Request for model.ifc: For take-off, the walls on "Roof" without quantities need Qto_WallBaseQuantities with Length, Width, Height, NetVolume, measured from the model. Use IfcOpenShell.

First a look at what the model holds.

```python
import ifcopenshell
import ifcopenshell.util.element
import ifcopenshell.util.unit

model = ifcopenshell.open("model.ifc")
print(model.schema)
for unit_type in ("LENGTHUNIT", "AREAUNIT", "VOLUMEUNIT"):
    print(unit_type, ifcopenshell.util.unit.calculate_unit_scale(model, unit_type))
storey = next(s for s in model.by_type("IfcBuildingStorey") if s.Name == "Roof")
walls = [e for e in ifcopenshell.util.element.get_decomposition(storey) if e.is_a("IfcWall")]
for e in sorted(walls, key=lambda e: e.id()):
    print(e.id(), e.is_a(), e.Name, list(ifcopenshell.util.element.get_psets(e, qtos_only=True)), sep=" | ")
```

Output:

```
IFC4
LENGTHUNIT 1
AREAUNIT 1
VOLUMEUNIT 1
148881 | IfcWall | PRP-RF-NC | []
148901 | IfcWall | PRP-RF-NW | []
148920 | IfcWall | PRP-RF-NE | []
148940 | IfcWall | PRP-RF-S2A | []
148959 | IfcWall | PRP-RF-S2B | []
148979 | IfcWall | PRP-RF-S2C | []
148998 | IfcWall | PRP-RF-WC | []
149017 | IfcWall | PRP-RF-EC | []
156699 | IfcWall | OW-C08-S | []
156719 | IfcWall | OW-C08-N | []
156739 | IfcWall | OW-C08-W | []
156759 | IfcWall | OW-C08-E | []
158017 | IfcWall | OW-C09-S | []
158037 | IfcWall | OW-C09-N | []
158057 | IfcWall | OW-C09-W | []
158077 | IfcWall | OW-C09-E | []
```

```python
import ifcopenshell
import ifcopenshell.api.pset
import ifcopenshell.geom
import ifcopenshell.util.element
import ifcopenshell.util.shape
import ifcopenshell.util.unit

model = ifcopenshell.open("model.ifc")
unit_scale = ifcopenshell.util.unit.calculate_unit_scale(model)
volume_scale = ifcopenshell.util.unit.calculate_unit_scale(model, "VOLUMEUNIT")
settings = ifcopenshell.geom.settings()

storey = next(s for s in model.by_type("IfcBuildingStorey") if s.Name == "Roof")
walls = [e for e in ifcopenshell.util.element.get_decomposition(storey) if e.is_a("IfcWall")]

for e in sorted(walls, key=lambda e: e.id()):
    if ifcopenshell.util.element.get_psets(e, qtos_only=True, should_inherit=False):
        continue
    # Geometry comes back in metres, in the element's own axes.
    shape = ifcopenshell.geom.create_shape(settings, e)
    values = {
        "Length": ifcopenshell.util.shape.get_x(shape.geometry) / unit_scale,
        "Width": ifcopenshell.util.shape.get_y(shape.geometry) / unit_scale,
        "Height": ifcopenshell.util.shape.get_z(shape.geometry) / unit_scale,
        "NetVolume": ifcopenshell.util.shape.get_volume(shape.geometry) / volume_scale,
    }
    qto = ifcopenshell.api.pset.add_qto(model, product=e, name="Qto_WallBaseQuantities")
    ifcopenshell.api.pset.edit_qto(model, qto=qto, properties=values)
    print(e.id(), {k: round(v, 3) for k, v in values.items()})

model.write("model-out.ifc")
```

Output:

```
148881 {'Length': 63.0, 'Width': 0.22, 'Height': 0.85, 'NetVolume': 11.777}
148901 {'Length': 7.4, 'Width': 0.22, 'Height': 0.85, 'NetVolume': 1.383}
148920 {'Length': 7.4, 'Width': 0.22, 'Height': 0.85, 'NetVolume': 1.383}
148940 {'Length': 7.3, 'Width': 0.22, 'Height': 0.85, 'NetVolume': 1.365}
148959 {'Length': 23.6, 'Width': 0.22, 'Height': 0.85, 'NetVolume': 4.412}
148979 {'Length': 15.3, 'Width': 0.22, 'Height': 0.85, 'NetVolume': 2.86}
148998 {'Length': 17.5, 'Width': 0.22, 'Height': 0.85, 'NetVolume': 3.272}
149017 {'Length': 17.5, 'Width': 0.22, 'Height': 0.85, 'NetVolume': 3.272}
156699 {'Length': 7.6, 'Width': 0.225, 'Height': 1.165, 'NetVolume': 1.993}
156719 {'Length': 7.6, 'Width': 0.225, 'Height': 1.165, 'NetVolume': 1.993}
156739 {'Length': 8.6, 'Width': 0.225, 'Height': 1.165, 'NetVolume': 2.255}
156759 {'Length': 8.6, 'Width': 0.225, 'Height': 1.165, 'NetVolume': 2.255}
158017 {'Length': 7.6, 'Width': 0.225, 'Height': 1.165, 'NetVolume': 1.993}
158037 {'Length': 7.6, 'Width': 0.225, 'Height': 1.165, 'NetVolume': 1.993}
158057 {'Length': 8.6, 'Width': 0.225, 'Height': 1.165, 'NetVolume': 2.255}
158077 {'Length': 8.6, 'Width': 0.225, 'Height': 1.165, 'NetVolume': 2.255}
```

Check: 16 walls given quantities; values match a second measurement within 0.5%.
